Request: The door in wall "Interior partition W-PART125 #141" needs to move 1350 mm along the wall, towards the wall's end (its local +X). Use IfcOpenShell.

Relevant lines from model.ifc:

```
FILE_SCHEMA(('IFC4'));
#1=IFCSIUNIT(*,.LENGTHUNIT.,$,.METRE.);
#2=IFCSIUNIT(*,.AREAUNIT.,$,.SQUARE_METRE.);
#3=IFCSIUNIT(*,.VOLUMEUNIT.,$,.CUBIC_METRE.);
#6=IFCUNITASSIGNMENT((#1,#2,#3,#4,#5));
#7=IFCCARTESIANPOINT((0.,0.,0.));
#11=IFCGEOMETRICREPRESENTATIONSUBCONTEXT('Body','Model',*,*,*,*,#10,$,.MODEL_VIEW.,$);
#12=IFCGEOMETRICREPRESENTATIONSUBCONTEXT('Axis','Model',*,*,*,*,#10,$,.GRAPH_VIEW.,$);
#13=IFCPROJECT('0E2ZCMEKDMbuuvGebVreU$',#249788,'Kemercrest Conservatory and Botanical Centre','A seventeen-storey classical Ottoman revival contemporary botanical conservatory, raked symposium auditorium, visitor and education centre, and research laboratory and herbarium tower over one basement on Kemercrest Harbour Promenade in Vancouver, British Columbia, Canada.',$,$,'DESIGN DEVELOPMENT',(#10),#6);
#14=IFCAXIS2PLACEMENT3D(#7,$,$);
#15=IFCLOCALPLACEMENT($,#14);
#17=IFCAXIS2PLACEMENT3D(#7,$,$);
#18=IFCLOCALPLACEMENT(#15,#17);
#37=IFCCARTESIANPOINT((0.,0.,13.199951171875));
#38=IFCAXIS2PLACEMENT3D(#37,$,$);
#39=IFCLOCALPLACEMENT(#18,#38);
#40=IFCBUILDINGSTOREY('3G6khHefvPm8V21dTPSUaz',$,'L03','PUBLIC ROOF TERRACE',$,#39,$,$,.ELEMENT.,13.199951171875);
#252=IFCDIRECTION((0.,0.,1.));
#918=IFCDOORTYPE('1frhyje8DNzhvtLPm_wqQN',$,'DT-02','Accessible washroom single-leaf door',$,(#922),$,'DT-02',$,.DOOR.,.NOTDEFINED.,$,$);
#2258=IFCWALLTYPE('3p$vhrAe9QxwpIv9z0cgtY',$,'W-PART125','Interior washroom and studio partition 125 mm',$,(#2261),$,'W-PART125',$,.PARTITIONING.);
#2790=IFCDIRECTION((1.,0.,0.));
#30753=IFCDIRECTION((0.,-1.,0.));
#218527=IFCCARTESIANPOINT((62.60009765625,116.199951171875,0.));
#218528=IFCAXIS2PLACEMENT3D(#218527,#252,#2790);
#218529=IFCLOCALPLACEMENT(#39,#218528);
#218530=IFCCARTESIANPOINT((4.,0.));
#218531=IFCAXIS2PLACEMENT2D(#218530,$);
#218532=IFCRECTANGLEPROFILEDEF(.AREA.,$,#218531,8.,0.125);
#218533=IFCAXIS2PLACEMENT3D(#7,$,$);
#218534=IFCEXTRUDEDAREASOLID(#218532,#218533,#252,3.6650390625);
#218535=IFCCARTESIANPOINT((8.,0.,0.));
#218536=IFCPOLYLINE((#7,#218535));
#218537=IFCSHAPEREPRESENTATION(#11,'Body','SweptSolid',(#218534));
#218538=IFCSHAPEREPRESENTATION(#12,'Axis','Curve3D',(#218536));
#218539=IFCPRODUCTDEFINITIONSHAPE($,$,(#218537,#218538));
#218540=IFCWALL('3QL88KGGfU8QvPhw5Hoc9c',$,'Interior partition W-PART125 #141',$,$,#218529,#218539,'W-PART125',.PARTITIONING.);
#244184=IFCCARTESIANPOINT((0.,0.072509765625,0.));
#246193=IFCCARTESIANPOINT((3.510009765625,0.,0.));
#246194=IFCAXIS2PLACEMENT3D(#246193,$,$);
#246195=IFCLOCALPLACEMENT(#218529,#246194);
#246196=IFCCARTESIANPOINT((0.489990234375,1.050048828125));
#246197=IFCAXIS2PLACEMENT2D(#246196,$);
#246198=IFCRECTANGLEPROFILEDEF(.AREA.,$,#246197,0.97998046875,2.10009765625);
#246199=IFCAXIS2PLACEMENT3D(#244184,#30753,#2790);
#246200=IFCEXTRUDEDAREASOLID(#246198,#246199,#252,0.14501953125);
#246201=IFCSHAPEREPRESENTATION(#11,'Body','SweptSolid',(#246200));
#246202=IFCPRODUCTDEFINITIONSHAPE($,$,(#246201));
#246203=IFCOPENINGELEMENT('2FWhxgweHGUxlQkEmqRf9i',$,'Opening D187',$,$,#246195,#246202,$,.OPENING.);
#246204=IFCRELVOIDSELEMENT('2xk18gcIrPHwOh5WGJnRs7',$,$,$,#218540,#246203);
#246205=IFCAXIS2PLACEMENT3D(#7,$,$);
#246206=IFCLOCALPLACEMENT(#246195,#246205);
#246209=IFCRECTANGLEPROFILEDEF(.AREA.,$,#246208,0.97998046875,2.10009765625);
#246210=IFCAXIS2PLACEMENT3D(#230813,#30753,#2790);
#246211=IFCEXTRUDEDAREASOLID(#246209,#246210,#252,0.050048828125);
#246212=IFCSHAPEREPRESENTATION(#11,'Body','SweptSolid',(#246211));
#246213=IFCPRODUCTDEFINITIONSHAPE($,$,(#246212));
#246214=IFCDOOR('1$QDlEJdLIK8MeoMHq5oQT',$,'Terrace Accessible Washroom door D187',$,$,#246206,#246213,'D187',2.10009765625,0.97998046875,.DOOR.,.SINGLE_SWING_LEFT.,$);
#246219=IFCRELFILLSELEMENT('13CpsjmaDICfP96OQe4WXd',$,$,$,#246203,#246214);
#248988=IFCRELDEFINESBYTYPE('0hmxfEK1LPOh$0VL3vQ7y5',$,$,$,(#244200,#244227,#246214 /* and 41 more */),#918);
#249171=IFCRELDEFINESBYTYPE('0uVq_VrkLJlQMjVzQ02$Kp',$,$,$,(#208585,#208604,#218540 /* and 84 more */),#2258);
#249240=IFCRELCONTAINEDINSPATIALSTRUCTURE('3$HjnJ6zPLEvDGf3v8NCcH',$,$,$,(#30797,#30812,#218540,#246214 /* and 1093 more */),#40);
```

```python
import ifcopenshell
import ifcopenshell.api.geometry
import ifcopenshell.util.placement

model = ifcopenshell.open("model.ifc")

door = model.by_id(246214)
opening = door.FillsVoids[0].RelatingOpeningElement
wall = opening.VoidsElements[0].RelatingBuildingElement

wall_matrix = ifcopenshell.util.placement.get_local_placement(wall.ObjectPlacement)
shift = wall_matrix[:3, 0] * 1.35
before = ifcopenshell.util.placement.get_local_placement(door.ObjectPlacement)[:3, 3].copy()

# The door is placed relative to its opening, so it follows when the opening moves.
matrix = ifcopenshell.util.placement.get_local_placement(opening.ObjectPlacement)
matrix[:3, 3] += shift
ifcopenshell.api.geometry.edit_object_placement(
    model, product=opening, matrix=matrix, is_si=False, should_transform_children=True
)

after = ifcopenshell.util.placement.get_local_placement(door.ObjectPlacement)[:3, 3]
print("door moved by", (after - before).round(3) + 0.0)

model.write("model_v2.ifc")
```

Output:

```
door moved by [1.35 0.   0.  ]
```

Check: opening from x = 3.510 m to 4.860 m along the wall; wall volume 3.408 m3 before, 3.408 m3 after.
